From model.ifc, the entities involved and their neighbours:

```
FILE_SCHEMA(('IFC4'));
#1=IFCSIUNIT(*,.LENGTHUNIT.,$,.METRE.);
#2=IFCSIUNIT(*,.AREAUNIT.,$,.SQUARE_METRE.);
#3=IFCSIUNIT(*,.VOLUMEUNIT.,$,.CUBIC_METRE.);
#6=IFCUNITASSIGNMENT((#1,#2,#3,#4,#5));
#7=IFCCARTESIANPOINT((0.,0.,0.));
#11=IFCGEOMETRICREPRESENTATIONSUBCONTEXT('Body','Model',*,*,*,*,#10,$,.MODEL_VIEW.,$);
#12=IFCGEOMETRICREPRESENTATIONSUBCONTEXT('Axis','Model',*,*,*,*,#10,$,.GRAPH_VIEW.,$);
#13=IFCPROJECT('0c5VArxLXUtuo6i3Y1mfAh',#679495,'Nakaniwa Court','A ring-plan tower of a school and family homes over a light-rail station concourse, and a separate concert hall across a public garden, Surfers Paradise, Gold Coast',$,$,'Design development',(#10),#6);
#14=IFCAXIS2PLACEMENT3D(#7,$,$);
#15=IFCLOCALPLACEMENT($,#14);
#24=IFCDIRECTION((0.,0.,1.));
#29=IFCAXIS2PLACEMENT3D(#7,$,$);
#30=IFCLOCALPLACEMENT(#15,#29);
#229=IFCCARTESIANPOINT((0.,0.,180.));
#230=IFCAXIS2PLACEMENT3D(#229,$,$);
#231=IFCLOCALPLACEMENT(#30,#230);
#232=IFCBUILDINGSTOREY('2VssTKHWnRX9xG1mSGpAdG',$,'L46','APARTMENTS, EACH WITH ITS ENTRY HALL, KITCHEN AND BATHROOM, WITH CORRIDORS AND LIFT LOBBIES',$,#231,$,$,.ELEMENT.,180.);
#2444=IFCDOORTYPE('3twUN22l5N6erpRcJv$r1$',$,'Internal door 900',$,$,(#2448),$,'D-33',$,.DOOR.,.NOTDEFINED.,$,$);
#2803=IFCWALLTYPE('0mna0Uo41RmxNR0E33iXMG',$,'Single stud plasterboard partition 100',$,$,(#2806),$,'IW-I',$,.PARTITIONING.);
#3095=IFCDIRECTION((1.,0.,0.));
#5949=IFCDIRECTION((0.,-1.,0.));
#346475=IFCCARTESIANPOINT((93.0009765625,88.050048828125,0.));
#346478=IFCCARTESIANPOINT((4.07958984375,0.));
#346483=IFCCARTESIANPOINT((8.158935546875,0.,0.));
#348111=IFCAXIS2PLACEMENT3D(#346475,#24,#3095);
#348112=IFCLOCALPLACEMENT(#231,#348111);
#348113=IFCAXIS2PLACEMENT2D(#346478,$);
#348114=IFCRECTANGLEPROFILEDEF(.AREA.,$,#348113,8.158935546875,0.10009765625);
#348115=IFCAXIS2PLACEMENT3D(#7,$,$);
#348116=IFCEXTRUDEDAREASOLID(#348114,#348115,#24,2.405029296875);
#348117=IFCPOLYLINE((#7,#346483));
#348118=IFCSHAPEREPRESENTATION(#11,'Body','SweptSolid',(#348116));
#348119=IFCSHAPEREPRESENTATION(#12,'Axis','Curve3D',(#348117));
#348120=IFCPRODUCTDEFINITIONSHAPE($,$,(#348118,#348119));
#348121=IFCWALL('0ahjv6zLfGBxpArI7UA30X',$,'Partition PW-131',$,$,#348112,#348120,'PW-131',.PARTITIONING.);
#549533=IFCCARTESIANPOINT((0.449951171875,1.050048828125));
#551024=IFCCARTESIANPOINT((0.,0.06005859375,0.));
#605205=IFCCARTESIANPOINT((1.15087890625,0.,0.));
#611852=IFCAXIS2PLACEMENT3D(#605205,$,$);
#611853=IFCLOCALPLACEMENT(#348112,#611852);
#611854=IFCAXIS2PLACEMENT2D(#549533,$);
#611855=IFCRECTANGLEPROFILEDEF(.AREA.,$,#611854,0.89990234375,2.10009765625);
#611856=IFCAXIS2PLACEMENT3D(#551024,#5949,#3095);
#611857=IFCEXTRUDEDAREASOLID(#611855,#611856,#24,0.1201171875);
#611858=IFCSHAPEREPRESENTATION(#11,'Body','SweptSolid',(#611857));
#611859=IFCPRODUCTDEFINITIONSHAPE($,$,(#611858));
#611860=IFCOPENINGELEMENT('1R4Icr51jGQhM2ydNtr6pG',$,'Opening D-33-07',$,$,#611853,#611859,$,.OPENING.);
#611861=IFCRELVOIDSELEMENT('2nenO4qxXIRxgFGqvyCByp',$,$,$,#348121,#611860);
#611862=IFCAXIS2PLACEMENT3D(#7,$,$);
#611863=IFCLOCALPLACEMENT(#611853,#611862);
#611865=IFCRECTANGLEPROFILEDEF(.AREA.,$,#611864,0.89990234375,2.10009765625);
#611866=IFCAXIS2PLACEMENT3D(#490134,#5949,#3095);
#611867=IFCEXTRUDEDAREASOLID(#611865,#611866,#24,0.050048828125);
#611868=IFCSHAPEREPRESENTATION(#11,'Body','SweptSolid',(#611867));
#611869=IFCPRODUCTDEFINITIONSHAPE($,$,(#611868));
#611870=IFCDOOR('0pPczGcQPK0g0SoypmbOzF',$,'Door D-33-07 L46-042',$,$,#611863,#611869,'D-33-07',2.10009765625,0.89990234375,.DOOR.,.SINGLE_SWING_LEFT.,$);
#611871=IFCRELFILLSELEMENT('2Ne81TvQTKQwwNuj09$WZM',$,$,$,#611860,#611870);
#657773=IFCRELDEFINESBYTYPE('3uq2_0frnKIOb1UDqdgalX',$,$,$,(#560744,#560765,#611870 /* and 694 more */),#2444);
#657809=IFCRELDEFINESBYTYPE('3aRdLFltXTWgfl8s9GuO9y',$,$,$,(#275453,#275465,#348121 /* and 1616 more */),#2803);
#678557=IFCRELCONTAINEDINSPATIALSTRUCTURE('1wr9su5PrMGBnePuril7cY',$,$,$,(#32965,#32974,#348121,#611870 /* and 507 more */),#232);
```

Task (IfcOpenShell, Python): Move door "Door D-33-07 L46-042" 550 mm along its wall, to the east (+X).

```python
import ifcopenshell
import ifcopenshell.api.geometry
import ifcopenshell.util.placement

model = ifcopenshell.open("model.ifc")

door = model.by_guid("0pPczGcQPK0g0SoypmbOzF")
opening = door.FillsVoids[0].RelatingOpeningElement
wall = opening.VoidsElements[0].RelatingBuildingElement

wall_matrix = ifcopenshell.util.placement.get_local_placement(wall.ObjectPlacement)
shift = wall_matrix[:3, 0] * 0.55
before = ifcopenshell.util.placement.get_local_placement(door.ObjectPlacement)[:3, 3].copy()

# The door is placed relative to its opening, so it follows when the opening moves.
matrix = ifcopenshell.util.placement.get_local_placement(opening.ObjectPlacement)
matrix[:3, 3] += shift
ifcopenshell.api.geometry.edit_object_placement(
    model, product=opening, matrix=matrix, is_si=False, should_transform_children=True
)

after = ifcopenshell.util.placement.get_local_placement(door.ObjectPlacement)[:3, 3]
print("door moved by", (after - before).round(3) + 0.0)

model.write("model-out.ifc")
```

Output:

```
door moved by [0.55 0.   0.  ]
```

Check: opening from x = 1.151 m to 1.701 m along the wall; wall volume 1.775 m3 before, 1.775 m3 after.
